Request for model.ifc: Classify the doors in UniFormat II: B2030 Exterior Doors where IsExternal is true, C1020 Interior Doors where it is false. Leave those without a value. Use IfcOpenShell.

First a look at what the model holds.

```python
import ifcopenshell
import ifcopenshell.util.element

model = ifcopenshell.open("model.ifc")
print(model.schema)
print("classifications:", [c.Name for c in model.by_type("IfcClassification")])
values = [ifcopenshell.util.element.get_pset(e, "Pset_DoorCommon", "IsExternal") for e in model.by_type("IfcDoor")]
for value in (True, False, None):
    print("IsExternal", value, values.count(value))
```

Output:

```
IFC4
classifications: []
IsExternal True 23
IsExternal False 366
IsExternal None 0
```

```python
import ifcopenshell
import ifcopenshell.api.classification
import ifcopenshell.util.element

model = ifcopenshell.open("model.ifc")

system = ifcopenshell.api.classification.add_classification(model, classification="UniFormat II")

doors = model.by_type("IfcDoor")
external = {e: ifcopenshell.util.element.get_pset(e, "Pset_DoorCommon", "IsExternal") for e in doors}
for flag, code, name in ((True, "B2030", "Exterior Doors"), (False, "C1020", "Interior Doors")):
    products = [e for e in doors if external[e] is flag]
    ifcopenshell.api.classification.add_reference(
        model, products=products, classification=system, identification=code, name=name
    )
    print(code, len(products))

model.write("model-out.ifc")
```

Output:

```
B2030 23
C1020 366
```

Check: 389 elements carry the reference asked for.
